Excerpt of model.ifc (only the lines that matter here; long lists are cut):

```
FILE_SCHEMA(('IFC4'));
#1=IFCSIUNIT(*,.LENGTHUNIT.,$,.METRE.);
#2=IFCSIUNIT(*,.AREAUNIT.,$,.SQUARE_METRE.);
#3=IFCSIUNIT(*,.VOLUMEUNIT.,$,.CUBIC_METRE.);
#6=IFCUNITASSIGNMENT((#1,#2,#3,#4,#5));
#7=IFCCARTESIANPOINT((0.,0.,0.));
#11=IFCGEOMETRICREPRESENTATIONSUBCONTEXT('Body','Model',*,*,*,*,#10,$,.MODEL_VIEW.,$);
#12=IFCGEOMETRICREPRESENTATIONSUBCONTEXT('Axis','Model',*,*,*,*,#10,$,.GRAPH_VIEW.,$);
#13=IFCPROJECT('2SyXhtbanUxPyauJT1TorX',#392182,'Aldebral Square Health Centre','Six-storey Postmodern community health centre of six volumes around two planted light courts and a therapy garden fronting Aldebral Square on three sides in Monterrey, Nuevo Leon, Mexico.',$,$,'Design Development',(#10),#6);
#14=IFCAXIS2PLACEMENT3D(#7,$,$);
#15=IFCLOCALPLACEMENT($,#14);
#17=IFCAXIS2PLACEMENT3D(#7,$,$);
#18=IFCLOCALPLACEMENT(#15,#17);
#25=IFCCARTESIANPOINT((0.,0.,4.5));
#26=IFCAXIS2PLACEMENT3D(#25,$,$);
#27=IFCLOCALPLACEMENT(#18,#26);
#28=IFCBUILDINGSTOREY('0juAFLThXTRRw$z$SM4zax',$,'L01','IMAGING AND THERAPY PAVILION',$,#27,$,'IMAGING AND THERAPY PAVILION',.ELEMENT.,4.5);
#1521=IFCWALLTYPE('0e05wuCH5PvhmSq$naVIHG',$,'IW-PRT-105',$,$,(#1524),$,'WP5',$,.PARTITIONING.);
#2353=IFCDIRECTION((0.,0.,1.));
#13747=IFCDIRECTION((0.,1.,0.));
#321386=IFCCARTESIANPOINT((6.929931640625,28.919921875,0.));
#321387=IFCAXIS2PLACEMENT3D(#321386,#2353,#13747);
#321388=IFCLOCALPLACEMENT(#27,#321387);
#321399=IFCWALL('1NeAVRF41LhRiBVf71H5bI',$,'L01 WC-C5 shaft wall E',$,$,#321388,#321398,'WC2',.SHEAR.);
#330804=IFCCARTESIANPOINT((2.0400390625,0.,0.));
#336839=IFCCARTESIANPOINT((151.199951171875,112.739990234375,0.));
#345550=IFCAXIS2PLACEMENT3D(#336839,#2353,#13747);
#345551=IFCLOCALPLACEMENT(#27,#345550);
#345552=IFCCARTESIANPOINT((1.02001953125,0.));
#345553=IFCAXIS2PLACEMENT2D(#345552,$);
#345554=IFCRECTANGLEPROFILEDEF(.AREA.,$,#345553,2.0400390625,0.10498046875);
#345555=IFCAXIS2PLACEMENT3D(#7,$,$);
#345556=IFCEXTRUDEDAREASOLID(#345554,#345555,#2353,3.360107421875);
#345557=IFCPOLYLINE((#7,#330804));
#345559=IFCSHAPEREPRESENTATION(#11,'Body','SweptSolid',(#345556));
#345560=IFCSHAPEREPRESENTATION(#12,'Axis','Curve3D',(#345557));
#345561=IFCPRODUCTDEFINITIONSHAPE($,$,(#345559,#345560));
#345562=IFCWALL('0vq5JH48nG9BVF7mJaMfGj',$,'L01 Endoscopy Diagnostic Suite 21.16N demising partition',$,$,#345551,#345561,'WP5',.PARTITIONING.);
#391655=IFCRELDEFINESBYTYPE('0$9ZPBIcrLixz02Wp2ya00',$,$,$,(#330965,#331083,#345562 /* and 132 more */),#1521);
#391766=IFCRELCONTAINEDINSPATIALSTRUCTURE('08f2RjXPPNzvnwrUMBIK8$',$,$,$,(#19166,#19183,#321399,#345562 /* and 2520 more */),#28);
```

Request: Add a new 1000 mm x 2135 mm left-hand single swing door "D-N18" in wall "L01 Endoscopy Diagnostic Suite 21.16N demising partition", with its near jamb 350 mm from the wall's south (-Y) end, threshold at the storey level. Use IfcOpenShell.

```python
import numpy as np
import ifcopenshell
import ifcopenshell.api.feature
import ifcopenshell.api.geometry
import ifcopenshell.api.root
import ifcopenshell.api.spatial
import ifcopenshell.geom
import ifcopenshell.util.element
import ifcopenshell.util.placement
import ifcopenshell.util.representation
import ifcopenshell.util.shape
import ifcopenshell.util.unit

model = ifcopenshell.open("model.ifc")
unit_scale = ifcopenshell.util.unit.calculate_unit_scale(model)
settings = ifcopenshell.geom.settings()


def volume(element):
    """Net volume in cubic metres, openings subtracted."""
    shape = ifcopenshell.geom.create_shape(settings, element)
    return ifcopenshell.util.shape.get_volume(shape.geometry)


wall = model.by_guid("0vq5JH48nG9BVF7mJaMfGj")
storey = ifcopenshell.util.element.get_container(wall, ifc_class="IfcBuildingStorey")
context = ifcopenshell.util.representation.get_context(model, "Model", "Body", "MODEL_VIEW")
before = volume(wall)

width, height, from_end, sill = 1, 2.135, 0.35, 0.0  # metres

# The wall runs along its own X axis, and the end named is its -X end.
wall_shape = ifcopenshell.geom.create_shape(settings, wall)
x, y, z = ifcopenshell.util.shape.get_vertices(wall_shape.geometry).T
start = x.min() + from_end
face, thickness = float(y.min()), float(y.max() - y.min())
wall_matrix = ifcopenshell.util.placement.get_local_placement(wall.ObjectPlacement)
level = ifcopenshell.util.placement.get_local_placement(storey.ObjectPlacement)[2, 3]


def in_wall(x, y):
    """Placement at x, y metres in the wall's axes, at sill height."""
    matrix = wall_matrix.copy()
    matrix[:, 3] = wall_matrix @ np.array([x / unit_scale, y / unit_scale, 0.0, 1.0])
    matrix[2, 3] = level + sill / unit_scale
    return matrix


# Opening: a box that overshoots both wall faces by 50 mm.
opening = ifcopenshell.api.root.create_entity(model, ifc_class="IfcOpeningElement", predefined_type="OPENING")
box = ifcopenshell.api.geometry.add_wall_representation(
    model, context=context, length=width, height=height, thickness=thickness + 0.1
)
ifcopenshell.api.geometry.assign_representation(model, product=opening, representation=box)
ifcopenshell.api.geometry.edit_object_placement(model, product=opening, matrix=in_wall(start, face - 0.05), is_si=False)
ifcopenshell.api.feature.add_feature(model, feature=opening, element=wall)

door = ifcopenshell.api.root.create_entity(model, ifc_class="IfcDoor", name="D-N18", predefined_type="DOOR")
door.OverallWidth, door.OverallHeight = width / unit_scale, height / unit_scale
door.OperationType = "SINGLE_SWING_LEFT"
body = ifcopenshell.api.geometry.add_door_representation(
    model,
    context=context,
    overall_width=door.OverallWidth,
    overall_height=door.OverallHeight,
    operation_type="SINGLE_SWING_LEFT",
    lining_properties={"LiningDepth": thickness / unit_scale, "ThresholdDepth": thickness / unit_scale},
)
ifcopenshell.api.geometry.assign_representation(model, product=door, representation=body)
ifcopenshell.api.spatial.assign_container(model, products=[door], relating_structure=storey)
ifcopenshell.api.feature.add_filling(model, opening=opening, element=door)

# The lining spans the wall, so the door starts at the wall face.
ifcopenshell.api.geometry.edit_object_placement(model, product=door, matrix=in_wall(start, face), is_si=False)

after = volume(wall)

print(f"wall volume {before:.3f} -> {after:.3f} m3")

model.write("model_edited.ifc")
```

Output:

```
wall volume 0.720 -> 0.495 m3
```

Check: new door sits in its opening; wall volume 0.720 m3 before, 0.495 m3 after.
